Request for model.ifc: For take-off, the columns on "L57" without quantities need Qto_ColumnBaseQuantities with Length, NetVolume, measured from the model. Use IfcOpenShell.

First a look at what the model holds.

```python
import ifcopenshell
import ifcopenshell.util.element
import ifcopenshell.util.unit

model = ifcopenshell.open("model.ifc")
print(model.schema)
for unit_type in ("LENGTHUNIT", "AREAUNIT", "VOLUMEUNIT"):
    print(unit_type, ifcopenshell.util.unit.calculate_unit_scale(model, unit_type))
storey = next(s for s in model.by_type("IfcBuildingStorey") if s.Name == "L57")
columns = [e for e in ifcopenshell.util.element.get_decomposition(storey) if e.is_a("IfcColumn")]
for e in sorted(columns, key=lambda e: e.id()):
    print(e.id(), e.is_a(), e.Name, list(ifcopenshell.util.element.get_psets(e, qtos_only=True)), sep=" | ")
```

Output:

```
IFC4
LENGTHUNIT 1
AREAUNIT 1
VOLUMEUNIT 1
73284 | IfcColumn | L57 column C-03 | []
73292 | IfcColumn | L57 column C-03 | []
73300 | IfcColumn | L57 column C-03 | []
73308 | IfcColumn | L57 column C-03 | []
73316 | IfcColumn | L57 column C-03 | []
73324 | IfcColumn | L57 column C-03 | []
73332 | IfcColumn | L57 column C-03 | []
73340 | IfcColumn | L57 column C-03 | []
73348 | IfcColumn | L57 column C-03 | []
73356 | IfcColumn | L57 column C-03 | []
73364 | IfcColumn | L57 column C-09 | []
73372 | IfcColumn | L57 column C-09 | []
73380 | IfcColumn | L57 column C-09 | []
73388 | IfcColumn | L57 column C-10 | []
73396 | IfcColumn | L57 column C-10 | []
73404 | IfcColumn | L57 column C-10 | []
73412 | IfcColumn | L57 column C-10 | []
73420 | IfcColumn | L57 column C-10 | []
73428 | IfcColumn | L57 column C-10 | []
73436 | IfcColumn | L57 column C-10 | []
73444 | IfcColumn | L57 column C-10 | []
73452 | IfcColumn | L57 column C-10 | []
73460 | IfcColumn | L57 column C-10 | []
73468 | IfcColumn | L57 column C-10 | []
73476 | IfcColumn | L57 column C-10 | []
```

```python
import ifcopenshell
import ifcopenshell.api.pset
import ifcopenshell.geom
import ifcopenshell.util.element
import ifcopenshell.util.shape
import ifcopenshell.util.unit

model = ifcopenshell.open("model.ifc")
unit_scale = ifcopenshell.util.unit.calculate_unit_scale(model)
volume_scale = ifcopenshell.util.unit.calculate_unit_scale(model, "VOLUMEUNIT")
settings = ifcopenshell.geom.settings()

storey = next(s for s in model.by_type("IfcBuildingStorey") if s.Name == "L57")
columns = [e for e in ifcopenshell.util.element.get_decomposition(storey) if e.is_a("IfcColumn")]

for e in sorted(columns, key=lambda e: e.id()):
    if ifcopenshell.util.element.get_psets(e, qtos_only=True, should_inherit=False):
        continue
    # Geometry comes back in metres, in the element's own axes.
    shape = ifcopenshell.geom.create_shape(settings, e)
    values = {
        "Length": ifcopenshell.util.shape.get_z(shape.geometry) / unit_scale,
        "NetVolume": ifcopenshell.util.shape.get_volume(shape.geometry) / volume_scale,
    }
    qto = ifcopenshell.api.pset.add_qto(model, product=e, name="Qto_ColumnBaseQuantities")
    ifcopenshell.api.pset.edit_qto(model, qto=qto, properties=values)
    print(e.id(), {k: round(v, 3) for k, v in values.items()})

model.write("model-out.ifc")
```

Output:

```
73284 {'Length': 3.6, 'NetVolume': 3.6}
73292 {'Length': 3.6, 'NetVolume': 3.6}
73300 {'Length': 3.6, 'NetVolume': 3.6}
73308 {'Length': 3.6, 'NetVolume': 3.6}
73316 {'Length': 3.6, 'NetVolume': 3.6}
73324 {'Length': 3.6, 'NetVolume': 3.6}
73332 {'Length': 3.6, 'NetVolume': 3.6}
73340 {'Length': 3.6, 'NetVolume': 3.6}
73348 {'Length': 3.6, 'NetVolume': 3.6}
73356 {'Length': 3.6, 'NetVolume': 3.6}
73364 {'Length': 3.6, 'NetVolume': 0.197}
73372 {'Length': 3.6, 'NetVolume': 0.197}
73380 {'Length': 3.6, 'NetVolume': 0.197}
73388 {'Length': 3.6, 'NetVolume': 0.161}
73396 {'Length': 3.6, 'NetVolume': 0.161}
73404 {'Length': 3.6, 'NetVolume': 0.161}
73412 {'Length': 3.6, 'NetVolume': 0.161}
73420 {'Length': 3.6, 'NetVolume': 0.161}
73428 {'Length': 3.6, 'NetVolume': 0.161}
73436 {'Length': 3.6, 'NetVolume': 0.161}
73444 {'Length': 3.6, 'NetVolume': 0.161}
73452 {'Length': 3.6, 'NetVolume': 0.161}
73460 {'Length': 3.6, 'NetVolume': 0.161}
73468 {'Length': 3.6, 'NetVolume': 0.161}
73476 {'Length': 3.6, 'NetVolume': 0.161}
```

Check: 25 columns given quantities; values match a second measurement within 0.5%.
